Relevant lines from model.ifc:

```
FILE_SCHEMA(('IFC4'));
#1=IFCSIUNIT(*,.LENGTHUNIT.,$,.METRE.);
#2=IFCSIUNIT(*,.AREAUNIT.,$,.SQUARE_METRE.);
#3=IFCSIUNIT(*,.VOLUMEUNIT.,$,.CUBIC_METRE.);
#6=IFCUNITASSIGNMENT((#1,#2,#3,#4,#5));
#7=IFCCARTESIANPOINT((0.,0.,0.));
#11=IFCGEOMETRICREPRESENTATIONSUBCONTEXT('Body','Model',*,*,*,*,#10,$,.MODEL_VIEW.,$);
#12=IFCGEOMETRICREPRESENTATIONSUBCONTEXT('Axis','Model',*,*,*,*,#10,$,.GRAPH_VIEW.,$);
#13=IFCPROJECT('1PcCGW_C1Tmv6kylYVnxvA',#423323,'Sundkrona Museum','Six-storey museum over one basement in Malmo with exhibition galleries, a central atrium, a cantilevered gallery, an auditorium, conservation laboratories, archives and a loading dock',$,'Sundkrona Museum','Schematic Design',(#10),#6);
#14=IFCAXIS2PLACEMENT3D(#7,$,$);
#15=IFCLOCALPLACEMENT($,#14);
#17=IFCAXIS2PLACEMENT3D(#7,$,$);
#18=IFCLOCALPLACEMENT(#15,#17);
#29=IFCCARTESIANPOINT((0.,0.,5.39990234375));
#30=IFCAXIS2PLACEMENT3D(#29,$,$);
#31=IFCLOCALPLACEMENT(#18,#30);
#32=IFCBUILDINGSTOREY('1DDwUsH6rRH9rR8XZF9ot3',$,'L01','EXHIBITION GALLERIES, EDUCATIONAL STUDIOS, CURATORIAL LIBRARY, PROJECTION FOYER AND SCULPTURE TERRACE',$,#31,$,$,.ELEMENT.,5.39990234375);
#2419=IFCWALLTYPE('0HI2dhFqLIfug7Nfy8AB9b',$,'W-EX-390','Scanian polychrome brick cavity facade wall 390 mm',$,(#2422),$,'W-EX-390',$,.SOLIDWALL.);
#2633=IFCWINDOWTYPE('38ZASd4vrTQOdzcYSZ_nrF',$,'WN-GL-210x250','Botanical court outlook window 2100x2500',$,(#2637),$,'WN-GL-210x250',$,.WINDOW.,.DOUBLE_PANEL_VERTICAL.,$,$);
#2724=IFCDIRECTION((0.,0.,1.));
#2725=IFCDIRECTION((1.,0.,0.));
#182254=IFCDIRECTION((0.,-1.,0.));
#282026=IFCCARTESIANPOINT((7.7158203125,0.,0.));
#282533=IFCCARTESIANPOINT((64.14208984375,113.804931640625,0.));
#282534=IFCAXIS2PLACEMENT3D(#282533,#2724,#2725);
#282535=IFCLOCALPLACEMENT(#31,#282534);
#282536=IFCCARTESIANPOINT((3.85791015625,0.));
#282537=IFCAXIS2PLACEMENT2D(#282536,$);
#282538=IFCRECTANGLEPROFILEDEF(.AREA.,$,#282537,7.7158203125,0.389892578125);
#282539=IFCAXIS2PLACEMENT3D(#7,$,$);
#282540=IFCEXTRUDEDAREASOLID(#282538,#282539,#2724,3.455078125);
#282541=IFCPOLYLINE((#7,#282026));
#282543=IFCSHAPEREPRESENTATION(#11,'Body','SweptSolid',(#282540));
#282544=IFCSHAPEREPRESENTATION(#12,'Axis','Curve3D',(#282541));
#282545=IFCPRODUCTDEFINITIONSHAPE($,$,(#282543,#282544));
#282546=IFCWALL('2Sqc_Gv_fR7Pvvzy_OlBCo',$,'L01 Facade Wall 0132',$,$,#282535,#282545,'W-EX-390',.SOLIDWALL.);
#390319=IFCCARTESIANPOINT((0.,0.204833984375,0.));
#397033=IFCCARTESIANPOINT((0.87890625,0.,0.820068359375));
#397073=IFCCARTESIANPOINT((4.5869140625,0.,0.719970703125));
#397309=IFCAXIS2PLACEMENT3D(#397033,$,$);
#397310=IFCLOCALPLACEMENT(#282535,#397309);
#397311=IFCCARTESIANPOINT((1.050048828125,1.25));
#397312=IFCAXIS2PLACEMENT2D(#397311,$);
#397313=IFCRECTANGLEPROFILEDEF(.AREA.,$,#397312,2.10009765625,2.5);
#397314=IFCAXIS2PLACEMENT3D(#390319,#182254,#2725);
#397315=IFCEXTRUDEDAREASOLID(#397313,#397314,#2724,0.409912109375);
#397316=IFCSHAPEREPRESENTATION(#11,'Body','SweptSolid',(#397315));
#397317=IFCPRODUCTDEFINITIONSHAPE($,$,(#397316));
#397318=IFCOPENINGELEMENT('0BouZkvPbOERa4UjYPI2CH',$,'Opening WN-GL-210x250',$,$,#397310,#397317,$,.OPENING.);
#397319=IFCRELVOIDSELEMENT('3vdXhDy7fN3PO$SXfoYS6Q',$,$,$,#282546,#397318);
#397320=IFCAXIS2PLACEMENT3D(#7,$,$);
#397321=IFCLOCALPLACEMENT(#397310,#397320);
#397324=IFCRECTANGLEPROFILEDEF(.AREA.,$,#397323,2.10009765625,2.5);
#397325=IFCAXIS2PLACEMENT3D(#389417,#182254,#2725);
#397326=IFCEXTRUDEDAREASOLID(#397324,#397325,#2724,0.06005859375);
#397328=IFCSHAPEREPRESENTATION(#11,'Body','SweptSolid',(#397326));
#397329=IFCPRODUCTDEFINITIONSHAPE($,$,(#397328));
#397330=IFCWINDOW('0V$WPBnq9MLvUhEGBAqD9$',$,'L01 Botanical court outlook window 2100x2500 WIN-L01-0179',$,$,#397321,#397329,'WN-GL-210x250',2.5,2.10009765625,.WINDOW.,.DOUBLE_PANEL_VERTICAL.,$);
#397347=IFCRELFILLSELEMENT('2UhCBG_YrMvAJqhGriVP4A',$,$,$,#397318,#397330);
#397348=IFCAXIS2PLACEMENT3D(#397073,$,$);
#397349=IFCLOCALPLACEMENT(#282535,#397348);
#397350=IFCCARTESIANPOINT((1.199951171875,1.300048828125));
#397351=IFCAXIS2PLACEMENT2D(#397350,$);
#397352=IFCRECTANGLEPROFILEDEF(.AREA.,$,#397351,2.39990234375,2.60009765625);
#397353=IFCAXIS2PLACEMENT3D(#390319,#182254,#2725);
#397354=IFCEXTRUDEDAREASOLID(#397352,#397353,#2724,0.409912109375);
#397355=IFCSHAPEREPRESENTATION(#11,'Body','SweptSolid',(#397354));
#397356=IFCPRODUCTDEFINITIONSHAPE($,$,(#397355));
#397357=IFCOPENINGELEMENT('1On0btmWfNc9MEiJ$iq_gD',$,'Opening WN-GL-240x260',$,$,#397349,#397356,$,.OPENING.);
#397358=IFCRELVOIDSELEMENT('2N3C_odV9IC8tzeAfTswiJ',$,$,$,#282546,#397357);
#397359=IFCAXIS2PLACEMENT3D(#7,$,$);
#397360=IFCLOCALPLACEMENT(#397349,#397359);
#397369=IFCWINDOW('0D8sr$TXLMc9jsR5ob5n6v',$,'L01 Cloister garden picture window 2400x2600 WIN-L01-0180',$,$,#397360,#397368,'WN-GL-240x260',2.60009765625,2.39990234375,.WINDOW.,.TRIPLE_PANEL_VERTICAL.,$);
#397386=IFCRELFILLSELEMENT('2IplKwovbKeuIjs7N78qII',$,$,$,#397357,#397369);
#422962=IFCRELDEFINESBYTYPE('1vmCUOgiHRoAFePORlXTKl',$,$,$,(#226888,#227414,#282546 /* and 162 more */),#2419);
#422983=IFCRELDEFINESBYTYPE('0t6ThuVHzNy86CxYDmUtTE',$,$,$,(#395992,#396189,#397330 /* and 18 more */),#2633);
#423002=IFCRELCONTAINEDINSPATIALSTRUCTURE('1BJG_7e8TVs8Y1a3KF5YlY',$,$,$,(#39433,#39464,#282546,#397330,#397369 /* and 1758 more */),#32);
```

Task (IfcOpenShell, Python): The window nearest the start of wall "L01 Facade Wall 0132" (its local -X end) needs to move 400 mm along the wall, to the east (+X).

```python
import ifcopenshell
import ifcopenshell.api.geometry
import ifcopenshell.util.placement
import ifcopenshell.util.unit

model = ifcopenshell.open("model.ifc")
unit_scale = ifcopenshell.util.unit.calculate_unit_scale(model)

window = model.by_guid("0V$WPBnq9MLvUhEGBAqD9$")
opening = window.FillsVoids[0].RelatingOpeningElement
wall = opening.VoidsElements[0].RelatingBuildingElement

wall_matrix = ifcopenshell.util.placement.get_local_placement(wall.ObjectPlacement)
shift = wall_matrix[:3, 0] * 0.4 / unit_scale
before = ifcopenshell.util.placement.get_local_placement(window.ObjectPlacement)[:3, 3].copy()

# The window is placed relative to its opening, so it follows when the opening moves.
matrix = ifcopenshell.util.placement.get_local_placement(opening.ObjectPlacement)
matrix[:3, 3] += shift
ifcopenshell.api.geometry.edit_object_placement(
    model, product=opening, matrix=matrix, is_si=False, should_transform_children=True
)

after = ifcopenshell.util.placement.get_local_placement(window.ObjectPlacement)[:3, 3]
print("window moved by", (after - before).round(3) + 0.0)

model.write("model_edited.ifc")
```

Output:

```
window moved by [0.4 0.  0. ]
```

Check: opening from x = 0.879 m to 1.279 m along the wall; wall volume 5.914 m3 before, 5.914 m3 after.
